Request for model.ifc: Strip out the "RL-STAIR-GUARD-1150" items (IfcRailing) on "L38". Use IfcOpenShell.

First a look at what the model holds.

```python
import ifcopenshell
import ifcopenshell.util.element

model = ifcopenshell.open("model.ifc")
print(model.schema)
storey = next(s for s in model.by_type("IfcBuildingStorey") if s.Name == "L38")
railings = [e for e in ifcopenshell.util.element.get_decomposition(storey) if e.is_a("IfcRailing")]
seen = {}
for e in railings:
    element_type = ifcopenshell.util.element.get_type(e)
    name = element_type.Name if element_type not in (None, e) else None
    seen[name] = seen.get(name, 0) + 1
for name, count in sorted(seen.items(), key=str):
    print(count, "x", name)
```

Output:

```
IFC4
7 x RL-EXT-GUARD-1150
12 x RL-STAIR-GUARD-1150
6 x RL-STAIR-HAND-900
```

```python
import ifcopenshell
import ifcopenshell.api.root
import ifcopenshell.util.element

model = ifcopenshell.open("model.ifc")

storey = next(s for s in model.by_type("IfcBuildingStorey") if s.Name == "L38")
railings = [e for e in ifcopenshell.util.element.get_decomposition(storey) if e.is_a("IfcRailing")]
targets = [e for e in railings if (t := ifcopenshell.util.element.get_type(e)) not in (None, e) and t.Name == "RL-STAIR-GUARD-1150"]

for e in targets:
    ifcopenshell.api.root.remove_product(model, product=e)
print(len(targets), "removed")

model.write("model_updated.ifc")
```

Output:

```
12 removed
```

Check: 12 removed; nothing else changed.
